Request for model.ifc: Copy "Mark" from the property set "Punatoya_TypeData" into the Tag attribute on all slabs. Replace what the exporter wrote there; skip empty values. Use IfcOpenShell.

First a look at what the model holds.

```python
import ifcopenshell
import ifcopenshell.util.element

model = ifcopenshell.open("model.ifc")
print(model.schema)
slabs = model.by_type("IfcSlab")
print(len(slabs), "slabs")
for e in slabs[:8]:
    source = ifcopenshell.util.element.get_pset(e, "Punatoya_TypeData", "Mark")
    target = e.Tag
    print(e.id(), repr(source), repr(target), sep=" | ")
```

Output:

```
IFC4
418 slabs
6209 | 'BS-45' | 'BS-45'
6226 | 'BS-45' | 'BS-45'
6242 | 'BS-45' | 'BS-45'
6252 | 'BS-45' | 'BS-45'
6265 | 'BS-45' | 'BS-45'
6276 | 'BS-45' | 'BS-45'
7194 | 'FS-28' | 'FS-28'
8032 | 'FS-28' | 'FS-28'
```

```python
import ifcopenshell
import ifcopenshell.util.element

model = ifcopenshell.open("model.ifc")

count = 0
for e in model.by_type("IfcSlab"):
    value = ifcopenshell.util.element.get_pset(e, "Punatoya_TypeData", "Mark")
    current = e.Tag
    if not value or not value.strip() or current == value:
        continue
    e.Tag = value
    count += 1

print(count, "slabs updated")

model.write("model_v2.ifc")
```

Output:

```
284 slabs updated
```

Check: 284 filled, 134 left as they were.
